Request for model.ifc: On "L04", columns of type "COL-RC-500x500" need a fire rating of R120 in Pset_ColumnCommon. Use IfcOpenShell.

First a look at what the model holds.

```python
import ifcopenshell
import ifcopenshell.util.element

model = ifcopenshell.open("model.ifc")
print(model.schema)
storey = next(s for s in model.by_type("IfcBuildingStorey") if s.Name == "L04")
columns = [e for e in ifcopenshell.util.element.get_decomposition(storey) if e.is_a("IfcColumn")]
seen = {}
for e in columns:
    element_type = ifcopenshell.util.element.get_type(e)
    key = (element_type.Name if element_type != e and element_type else None, ifcopenshell.util.element.get_pset(e, "Pset_ColumnCommon", "FireRating"))
    seen[key] = seen.get(key, 0) + 1
for (name, value), count in sorted(seen.items(), key=str):
    print(count, "x", name, "|", value)
```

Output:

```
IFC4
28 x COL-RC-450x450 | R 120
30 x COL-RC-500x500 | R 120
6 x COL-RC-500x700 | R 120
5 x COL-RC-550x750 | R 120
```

```python
import ifcopenshell
import ifcopenshell.api.pset
import ifcopenshell.util.element

model = ifcopenshell.open("model.ifc")

storey = next(s for s in model.by_type("IfcBuildingStorey") if s.Name == "L04")
columns = [e for e in ifcopenshell.util.element.get_decomposition(storey) if e.is_a("IfcColumn")]

count = 0
for e in columns:
    element_type = ifcopenshell.util.element.get_type(e)
    if element_type in (None, e) or element_type.Name != "COL-RC-500x500":
        continue
    # add_pset returns the element's existing set when there is one.
    pset = ifcopenshell.api.pset.add_pset(model, product=e, name="Pset_ColumnCommon")
    ifcopenshell.api.pset.edit_pset(model, pset=pset, properties={"FireRating": "R120"})
    count += 1

print(count, "columns updated")

model.write("model_edited.ifc")
```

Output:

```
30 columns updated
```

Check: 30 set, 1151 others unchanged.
